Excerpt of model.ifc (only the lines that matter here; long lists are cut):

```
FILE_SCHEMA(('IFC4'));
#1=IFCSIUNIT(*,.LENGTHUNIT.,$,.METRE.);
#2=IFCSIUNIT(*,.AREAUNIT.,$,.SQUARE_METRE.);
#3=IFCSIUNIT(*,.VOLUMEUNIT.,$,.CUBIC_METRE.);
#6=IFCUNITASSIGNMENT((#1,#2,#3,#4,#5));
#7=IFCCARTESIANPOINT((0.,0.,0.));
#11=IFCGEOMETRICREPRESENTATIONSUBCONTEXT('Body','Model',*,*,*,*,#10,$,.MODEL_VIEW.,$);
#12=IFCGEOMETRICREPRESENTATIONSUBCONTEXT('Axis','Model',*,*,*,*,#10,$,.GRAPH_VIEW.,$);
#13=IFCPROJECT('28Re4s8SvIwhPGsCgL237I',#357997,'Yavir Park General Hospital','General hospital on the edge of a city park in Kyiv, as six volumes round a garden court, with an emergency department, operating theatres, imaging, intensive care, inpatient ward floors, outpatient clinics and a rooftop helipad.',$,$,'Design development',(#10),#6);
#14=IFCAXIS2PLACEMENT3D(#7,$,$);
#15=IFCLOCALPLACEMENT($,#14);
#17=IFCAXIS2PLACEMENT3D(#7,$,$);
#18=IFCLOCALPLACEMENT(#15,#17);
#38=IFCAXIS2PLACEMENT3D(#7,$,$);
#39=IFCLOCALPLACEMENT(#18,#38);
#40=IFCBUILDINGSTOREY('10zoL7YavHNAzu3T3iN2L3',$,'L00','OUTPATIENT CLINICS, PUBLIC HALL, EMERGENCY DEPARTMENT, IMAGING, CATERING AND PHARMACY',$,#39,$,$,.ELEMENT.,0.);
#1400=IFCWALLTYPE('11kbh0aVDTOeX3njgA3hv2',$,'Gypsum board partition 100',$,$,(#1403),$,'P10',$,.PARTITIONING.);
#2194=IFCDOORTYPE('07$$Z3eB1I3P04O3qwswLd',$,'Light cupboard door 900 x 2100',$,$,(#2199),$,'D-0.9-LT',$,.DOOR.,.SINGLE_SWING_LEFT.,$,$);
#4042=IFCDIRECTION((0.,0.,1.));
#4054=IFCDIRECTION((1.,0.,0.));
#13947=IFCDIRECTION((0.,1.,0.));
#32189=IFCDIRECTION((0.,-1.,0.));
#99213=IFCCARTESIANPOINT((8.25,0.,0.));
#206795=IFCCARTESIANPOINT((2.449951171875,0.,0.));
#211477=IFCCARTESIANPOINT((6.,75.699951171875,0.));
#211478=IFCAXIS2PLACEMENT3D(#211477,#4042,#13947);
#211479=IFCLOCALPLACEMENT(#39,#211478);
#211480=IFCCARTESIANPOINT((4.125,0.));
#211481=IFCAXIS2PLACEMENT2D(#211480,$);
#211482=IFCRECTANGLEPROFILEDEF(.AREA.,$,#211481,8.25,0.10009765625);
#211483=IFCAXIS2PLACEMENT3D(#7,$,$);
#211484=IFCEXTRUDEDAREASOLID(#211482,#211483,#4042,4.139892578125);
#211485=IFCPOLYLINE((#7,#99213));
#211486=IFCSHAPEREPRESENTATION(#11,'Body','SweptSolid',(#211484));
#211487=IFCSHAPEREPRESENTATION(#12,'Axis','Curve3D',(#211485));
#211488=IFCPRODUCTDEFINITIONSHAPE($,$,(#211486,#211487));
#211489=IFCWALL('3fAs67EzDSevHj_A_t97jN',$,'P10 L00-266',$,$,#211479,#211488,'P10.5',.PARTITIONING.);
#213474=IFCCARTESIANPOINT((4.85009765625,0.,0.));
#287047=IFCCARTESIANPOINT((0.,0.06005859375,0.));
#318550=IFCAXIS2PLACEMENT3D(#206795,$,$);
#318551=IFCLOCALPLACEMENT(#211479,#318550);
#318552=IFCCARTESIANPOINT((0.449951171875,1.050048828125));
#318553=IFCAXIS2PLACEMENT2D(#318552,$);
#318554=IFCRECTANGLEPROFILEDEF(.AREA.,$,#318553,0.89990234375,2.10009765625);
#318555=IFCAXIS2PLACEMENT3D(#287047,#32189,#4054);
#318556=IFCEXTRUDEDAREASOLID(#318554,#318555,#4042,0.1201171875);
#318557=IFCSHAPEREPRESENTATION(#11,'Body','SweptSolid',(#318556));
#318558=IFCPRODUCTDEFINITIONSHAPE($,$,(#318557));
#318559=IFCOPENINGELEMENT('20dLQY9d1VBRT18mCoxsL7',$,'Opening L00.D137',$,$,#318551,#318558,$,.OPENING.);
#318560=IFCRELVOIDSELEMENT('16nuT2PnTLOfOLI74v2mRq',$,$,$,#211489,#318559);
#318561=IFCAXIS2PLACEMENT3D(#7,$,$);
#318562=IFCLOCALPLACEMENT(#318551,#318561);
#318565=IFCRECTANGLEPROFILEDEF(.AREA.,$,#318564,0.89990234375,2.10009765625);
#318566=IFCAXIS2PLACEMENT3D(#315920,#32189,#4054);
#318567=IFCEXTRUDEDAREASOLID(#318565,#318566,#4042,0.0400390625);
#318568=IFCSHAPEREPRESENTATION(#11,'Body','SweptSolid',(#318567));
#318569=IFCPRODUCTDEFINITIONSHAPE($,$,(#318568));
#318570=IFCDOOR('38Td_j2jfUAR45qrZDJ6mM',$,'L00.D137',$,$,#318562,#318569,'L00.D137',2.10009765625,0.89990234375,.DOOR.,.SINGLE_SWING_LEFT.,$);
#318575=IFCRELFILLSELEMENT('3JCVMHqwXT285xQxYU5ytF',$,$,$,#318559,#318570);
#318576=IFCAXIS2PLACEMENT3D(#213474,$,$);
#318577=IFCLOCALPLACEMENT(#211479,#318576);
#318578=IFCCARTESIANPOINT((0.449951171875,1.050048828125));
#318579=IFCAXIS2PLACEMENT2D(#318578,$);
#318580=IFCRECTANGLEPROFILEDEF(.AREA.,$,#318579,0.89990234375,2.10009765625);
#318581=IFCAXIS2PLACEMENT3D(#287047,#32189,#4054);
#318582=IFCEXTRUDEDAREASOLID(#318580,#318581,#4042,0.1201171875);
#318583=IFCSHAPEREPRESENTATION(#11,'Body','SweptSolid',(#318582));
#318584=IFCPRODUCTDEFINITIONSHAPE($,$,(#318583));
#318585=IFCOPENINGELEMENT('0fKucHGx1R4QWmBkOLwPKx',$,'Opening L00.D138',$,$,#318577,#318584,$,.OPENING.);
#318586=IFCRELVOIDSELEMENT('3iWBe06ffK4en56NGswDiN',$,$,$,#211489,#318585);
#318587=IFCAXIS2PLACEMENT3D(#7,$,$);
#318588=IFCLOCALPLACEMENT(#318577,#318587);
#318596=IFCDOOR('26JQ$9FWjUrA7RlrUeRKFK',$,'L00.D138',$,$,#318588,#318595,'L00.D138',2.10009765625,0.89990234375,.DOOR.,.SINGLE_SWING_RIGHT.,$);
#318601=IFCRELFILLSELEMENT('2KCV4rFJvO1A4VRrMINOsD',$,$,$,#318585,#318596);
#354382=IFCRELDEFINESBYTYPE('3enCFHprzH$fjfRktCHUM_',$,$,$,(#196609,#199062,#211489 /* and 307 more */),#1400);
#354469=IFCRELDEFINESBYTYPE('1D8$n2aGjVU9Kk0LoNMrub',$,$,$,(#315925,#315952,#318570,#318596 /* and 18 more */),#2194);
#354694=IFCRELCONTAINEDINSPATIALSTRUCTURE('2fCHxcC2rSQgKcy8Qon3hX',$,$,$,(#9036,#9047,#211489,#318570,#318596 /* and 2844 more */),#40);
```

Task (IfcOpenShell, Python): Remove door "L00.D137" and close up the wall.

```python
import ifcopenshell
import ifcopenshell.api.feature
import ifcopenshell.api.root
import ifcopenshell.geom
import ifcopenshell.util.shape

model = ifcopenshell.open("model.ifc")
settings = ifcopenshell.geom.settings()


def volume(element):
    """Net volume in cubic metres, openings subtracted."""
    shape = ifcopenshell.geom.create_shape(settings, element)
    return ifcopenshell.util.shape.get_volume(shape.geometry)


door = model.by_id(318570)
opening = door.FillsVoids[0].RelatingOpeningElement
wall = opening.VoidsElements[0].RelatingBuildingElement
before = volume(wall)

ifcopenshell.api.root.remove_product(model, product=door)
ifcopenshell.api.feature.remove_feature(model, feature=opening)

after = volume(wall)

print(f"wall volume {before:.3f} -> {after:.3f} m3")

model.write("model-out.ifc")
```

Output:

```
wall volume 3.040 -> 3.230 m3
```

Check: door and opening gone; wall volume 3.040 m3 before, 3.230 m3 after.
